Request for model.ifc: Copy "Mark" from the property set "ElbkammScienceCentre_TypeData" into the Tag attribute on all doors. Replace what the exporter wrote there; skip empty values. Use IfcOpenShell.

First a look at what the model holds.

```python
import ifcopenshell
import ifcopenshell.util.element

model = ifcopenshell.open("model.ifc")
print(model.schema)
doors = model.by_type("IfcDoor")
print(len(doors), "doors")
for e in doors[:8]:
    source = ifcopenshell.util.element.get_pset(e, "ElbkammScienceCentre_TypeData", "Mark")
    target = e.Tag
    print(e.id(), repr(source), repr(target), sep=" | ")
```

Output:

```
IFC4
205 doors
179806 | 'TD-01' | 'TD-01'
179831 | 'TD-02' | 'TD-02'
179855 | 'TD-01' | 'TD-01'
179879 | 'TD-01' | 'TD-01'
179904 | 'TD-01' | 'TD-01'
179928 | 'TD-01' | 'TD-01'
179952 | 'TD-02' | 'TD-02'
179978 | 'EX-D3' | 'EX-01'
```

```python
import ifcopenshell
import ifcopenshell.util.element

model = ifcopenshell.open("model.ifc")

count = 0
for e in model.by_type("IfcDoor"):
    value = ifcopenshell.util.element.get_pset(e, "ElbkammScienceCentre_TypeData", "Mark")
    current = e.Tag
    if not value or not value.strip() or current == value:
        continue
    e.Tag = value
    count += 1

print(count, "doors updated")

model.write("model-out.ifc")
```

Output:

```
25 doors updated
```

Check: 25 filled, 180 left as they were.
